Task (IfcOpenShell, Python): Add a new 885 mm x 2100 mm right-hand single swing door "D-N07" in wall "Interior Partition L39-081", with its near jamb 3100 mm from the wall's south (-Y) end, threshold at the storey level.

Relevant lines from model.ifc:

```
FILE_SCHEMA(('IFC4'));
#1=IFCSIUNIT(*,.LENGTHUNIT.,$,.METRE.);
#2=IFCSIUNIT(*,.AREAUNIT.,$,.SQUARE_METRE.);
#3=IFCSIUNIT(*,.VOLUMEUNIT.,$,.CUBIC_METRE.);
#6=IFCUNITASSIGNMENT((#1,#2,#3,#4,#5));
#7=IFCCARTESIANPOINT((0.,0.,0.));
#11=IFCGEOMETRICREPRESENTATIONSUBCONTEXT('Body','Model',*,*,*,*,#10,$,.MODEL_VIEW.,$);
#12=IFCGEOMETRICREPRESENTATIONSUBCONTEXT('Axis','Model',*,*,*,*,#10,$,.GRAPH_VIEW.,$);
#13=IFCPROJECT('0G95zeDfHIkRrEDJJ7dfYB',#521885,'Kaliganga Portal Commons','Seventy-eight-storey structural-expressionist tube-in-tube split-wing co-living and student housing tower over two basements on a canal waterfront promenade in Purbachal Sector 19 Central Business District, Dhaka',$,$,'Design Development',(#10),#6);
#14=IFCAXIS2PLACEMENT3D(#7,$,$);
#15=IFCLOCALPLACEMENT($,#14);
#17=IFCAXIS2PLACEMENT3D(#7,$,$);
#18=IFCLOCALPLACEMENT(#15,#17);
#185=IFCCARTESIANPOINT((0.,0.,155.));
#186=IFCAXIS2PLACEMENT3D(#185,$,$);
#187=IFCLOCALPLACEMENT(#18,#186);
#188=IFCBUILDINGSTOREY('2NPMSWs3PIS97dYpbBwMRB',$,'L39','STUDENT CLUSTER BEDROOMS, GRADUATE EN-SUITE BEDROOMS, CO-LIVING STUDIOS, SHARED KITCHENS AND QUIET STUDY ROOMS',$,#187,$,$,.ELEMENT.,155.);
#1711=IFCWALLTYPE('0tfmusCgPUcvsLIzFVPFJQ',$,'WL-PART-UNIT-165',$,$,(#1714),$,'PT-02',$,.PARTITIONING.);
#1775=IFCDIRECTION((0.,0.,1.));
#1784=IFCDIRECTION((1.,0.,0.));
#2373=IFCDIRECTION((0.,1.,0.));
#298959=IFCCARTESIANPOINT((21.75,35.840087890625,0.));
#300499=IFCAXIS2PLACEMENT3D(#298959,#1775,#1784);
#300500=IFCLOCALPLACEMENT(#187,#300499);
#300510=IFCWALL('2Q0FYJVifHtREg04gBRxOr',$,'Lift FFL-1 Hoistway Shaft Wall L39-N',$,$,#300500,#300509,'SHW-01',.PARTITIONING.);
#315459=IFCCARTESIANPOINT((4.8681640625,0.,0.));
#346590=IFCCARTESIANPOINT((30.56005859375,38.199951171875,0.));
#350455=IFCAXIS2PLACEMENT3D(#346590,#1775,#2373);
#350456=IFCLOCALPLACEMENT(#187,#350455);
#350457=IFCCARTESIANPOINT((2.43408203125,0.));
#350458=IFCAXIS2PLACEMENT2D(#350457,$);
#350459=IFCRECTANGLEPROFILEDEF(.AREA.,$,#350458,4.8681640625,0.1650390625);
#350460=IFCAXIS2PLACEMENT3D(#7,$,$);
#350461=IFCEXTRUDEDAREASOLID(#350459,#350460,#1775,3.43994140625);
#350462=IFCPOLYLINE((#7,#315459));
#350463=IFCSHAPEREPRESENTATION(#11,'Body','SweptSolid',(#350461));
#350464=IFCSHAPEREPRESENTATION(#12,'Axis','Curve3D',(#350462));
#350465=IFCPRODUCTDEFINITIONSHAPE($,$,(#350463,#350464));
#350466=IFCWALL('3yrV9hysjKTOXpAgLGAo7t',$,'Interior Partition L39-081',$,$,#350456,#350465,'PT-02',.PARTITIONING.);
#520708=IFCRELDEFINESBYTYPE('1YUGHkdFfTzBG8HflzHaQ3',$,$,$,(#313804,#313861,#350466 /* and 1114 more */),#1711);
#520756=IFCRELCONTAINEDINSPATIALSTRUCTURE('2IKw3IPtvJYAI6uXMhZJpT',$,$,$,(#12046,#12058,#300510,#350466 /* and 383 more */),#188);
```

```python
import numpy as np
import ifcopenshell
import ifcopenshell.api.feature
import ifcopenshell.api.geometry
import ifcopenshell.api.root
import ifcopenshell.api.spatial
import ifcopenshell.geom
import ifcopenshell.util.element
import ifcopenshell.util.placement
import ifcopenshell.util.representation
import ifcopenshell.util.shape
import ifcopenshell.util.unit

model = ifcopenshell.open("model.ifc")
unit_scale = ifcopenshell.util.unit.calculate_unit_scale(model)
settings = ifcopenshell.geom.settings()


def volume(element):
    """Net volume in cubic metres, openings subtracted."""
    shape = ifcopenshell.geom.create_shape(settings, element)
    return ifcopenshell.util.shape.get_volume(shape.geometry)


wall = model.by_guid("3yrV9hysjKTOXpAgLGAo7t")
storey = ifcopenshell.util.element.get_container(wall, ifc_class="IfcBuildingStorey")
context = ifcopenshell.util.representation.get_context(model, "Model", "Body", "MODEL_VIEW")
before = volume(wall)

width, height, from_end, sill = 0.885, 2.1, 3.1, 0.0  # metres

# The wall runs along its own X axis, and the end named is its -X end.
wall_shape = ifcopenshell.geom.create_shape(settings, wall)
x, y, z = ifcopenshell.util.shape.get_vertices(wall_shape.geometry).T
start = x.min() + from_end
face, thickness = float(y.min()), float(y.max() - y.min())
wall_matrix = ifcopenshell.util.placement.get_local_placement(wall.ObjectPlacement)
level = ifcopenshell.util.placement.get_local_placement(storey.ObjectPlacement)[2, 3]


def in_wall(x, y):
    """Placement at x, y metres in the wall's axes, at sill height."""
    matrix = wall_matrix.copy()
    matrix[:, 3] = wall_matrix @ np.array([x / unit_scale, y / unit_scale, 0.0, 1.0])
    matrix[2, 3] = level + sill / unit_scale
    return matrix


# Opening: a box that overshoots both wall faces by 50 mm.
opening = ifcopenshell.api.root.create_entity(model, ifc_class="IfcOpeningElement", predefined_type="OPENING")
box = ifcopenshell.api.geometry.add_wall_representation(
    model, context=context, length=width, height=height, thickness=thickness + 0.1
)
ifcopenshell.api.geometry.assign_representation(model, product=opening, representation=box)
ifcopenshell.api.geometry.edit_object_placement(model, product=opening, matrix=in_wall(start, face - 0.05), is_si=False)
ifcopenshell.api.feature.add_feature(model, feature=opening, element=wall)

door = ifcopenshell.api.root.create_entity(model, ifc_class="IfcDoor", name="D-N07", predefined_type="DOOR")
door.OverallWidth, door.OverallHeight = width / unit_scale, height / unit_scale
door.OperationType = "SINGLE_SWING_RIGHT"
body = ifcopenshell.api.geometry.add_door_representation(
    model,
    context=context,
    overall_width=door.OverallWidth,
    overall_height=door.OverallHeight,
    operation_type="SINGLE_SWING_RIGHT",
    lining_properties={"LiningDepth": thickness / unit_scale, "ThresholdDepth": thickness / unit_scale},
)
ifcopenshell.api.geometry.assign_representation(model, product=door, representation=body)
ifcopenshell.api.spatial.assign_container(model, products=[door], relating_structure=storey)
ifcopenshell.api.feature.add_filling(model, opening=opening, element=door)

# The lining spans the wall, so the door starts at the wall face.
ifcopenshell.api.geometry.edit_object_placement(model, product=door, matrix=in_wall(start, face), is_si=False)

after = volume(wall)

print(f"wall volume {before:.3f} -> {after:.3f} m3")

model.write("model-out.ifc")
```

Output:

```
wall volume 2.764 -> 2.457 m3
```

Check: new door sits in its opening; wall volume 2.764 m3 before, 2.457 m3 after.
